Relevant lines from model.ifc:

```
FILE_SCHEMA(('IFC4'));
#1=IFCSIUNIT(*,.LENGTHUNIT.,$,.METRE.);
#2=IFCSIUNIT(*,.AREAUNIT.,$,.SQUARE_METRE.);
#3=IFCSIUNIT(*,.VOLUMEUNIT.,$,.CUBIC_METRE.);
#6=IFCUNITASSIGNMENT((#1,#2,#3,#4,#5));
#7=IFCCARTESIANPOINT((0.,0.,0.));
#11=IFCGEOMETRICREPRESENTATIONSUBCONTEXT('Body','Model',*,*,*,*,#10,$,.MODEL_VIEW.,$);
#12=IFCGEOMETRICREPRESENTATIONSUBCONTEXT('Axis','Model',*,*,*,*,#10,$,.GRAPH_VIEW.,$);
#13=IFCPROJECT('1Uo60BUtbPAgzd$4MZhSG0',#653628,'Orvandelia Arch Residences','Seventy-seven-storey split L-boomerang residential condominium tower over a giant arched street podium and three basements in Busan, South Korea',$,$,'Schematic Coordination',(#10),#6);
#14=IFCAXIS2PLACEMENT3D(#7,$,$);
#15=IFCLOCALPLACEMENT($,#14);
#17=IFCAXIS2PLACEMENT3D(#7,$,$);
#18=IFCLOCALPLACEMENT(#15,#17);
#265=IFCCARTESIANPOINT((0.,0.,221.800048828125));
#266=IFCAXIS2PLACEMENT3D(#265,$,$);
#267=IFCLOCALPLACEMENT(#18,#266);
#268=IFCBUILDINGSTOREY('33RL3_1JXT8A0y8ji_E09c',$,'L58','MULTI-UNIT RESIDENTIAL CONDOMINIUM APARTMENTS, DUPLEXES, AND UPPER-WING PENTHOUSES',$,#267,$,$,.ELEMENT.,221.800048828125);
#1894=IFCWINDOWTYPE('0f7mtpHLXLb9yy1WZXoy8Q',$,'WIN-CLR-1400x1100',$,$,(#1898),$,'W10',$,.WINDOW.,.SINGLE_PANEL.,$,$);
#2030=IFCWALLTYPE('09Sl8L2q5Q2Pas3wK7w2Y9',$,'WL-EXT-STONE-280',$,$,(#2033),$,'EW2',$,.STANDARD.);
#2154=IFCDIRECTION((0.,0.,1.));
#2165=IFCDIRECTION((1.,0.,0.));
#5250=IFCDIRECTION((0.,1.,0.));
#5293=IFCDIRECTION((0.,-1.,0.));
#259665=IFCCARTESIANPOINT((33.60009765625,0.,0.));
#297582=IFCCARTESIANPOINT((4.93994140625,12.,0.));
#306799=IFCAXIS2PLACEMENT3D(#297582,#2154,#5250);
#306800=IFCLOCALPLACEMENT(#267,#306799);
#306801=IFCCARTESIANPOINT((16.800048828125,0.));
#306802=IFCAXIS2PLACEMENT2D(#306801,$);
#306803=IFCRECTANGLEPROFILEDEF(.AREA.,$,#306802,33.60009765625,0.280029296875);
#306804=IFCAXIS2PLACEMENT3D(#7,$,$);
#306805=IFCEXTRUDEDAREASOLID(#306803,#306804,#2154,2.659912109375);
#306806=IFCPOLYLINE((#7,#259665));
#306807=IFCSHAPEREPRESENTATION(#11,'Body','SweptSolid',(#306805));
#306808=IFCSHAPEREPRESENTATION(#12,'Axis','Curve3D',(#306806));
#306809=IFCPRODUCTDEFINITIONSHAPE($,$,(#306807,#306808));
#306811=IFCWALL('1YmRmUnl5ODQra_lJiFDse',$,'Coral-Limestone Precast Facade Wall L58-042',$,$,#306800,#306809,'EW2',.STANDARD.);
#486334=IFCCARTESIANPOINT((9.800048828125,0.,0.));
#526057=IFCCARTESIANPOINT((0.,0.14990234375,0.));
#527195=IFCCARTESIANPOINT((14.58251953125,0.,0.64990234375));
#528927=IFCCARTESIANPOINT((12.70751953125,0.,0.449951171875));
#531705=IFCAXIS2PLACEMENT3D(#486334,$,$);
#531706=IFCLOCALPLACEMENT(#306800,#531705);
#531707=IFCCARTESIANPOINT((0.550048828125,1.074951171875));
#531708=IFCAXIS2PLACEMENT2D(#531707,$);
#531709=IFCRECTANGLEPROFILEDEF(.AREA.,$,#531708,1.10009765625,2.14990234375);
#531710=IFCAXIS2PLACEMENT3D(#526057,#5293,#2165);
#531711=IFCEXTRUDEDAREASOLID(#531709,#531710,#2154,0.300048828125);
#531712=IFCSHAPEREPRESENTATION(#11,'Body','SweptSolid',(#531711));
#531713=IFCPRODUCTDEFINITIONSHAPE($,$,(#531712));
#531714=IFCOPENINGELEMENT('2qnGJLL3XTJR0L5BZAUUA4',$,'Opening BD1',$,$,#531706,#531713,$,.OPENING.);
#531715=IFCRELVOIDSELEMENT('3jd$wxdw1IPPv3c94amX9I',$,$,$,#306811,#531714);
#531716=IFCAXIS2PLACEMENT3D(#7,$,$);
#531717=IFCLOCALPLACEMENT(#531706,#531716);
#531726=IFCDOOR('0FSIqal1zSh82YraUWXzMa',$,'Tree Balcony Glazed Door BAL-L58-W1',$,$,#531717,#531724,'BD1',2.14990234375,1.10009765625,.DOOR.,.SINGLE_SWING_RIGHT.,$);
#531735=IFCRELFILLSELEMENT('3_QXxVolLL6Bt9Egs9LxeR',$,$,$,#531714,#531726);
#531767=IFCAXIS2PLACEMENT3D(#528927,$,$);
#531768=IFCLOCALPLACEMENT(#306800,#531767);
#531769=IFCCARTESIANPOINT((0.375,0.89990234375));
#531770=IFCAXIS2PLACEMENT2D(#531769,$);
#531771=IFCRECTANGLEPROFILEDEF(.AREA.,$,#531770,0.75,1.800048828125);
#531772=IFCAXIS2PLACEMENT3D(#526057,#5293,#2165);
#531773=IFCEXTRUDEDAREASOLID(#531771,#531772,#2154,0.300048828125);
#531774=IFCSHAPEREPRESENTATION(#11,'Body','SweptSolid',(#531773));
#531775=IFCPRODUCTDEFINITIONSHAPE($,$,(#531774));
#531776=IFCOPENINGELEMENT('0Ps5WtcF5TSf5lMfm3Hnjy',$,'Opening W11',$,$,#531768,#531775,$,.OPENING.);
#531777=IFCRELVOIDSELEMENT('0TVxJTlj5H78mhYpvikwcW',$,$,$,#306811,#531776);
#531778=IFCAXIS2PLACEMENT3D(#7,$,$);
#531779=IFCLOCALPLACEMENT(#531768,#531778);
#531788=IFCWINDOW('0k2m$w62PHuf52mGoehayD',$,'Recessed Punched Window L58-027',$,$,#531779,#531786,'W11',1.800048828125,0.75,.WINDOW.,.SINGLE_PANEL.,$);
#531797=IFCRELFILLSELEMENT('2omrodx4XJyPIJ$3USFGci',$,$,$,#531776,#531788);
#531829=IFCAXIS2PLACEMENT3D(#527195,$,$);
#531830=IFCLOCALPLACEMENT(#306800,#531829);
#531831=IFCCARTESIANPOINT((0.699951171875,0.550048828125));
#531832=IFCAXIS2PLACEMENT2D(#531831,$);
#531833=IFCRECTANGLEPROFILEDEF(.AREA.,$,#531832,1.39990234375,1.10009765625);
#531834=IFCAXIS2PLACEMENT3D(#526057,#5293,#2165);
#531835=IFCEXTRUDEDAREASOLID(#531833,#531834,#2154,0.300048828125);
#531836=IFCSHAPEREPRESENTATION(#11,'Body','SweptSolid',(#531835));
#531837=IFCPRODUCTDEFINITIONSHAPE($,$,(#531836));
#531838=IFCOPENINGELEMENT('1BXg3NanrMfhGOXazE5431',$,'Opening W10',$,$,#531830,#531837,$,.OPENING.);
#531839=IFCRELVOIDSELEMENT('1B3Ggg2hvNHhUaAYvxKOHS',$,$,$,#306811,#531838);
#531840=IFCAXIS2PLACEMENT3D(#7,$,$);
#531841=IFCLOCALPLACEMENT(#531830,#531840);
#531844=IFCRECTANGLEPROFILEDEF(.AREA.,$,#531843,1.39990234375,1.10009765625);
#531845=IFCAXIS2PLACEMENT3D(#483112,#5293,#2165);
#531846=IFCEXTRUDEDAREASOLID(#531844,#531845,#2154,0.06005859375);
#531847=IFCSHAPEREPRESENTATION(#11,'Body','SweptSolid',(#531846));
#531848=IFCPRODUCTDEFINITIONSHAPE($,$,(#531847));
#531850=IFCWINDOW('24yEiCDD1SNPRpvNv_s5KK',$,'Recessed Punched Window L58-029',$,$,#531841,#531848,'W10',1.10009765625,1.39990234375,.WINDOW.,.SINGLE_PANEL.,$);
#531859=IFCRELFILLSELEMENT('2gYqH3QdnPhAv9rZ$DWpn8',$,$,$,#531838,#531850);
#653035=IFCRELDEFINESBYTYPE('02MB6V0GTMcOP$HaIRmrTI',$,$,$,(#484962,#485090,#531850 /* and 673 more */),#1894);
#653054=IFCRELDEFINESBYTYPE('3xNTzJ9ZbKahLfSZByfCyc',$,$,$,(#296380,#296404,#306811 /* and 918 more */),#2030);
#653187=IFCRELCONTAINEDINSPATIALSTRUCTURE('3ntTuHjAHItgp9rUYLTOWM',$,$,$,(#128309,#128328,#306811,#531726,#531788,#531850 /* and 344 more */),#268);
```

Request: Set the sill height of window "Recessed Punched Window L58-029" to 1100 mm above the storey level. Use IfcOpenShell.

```python
import numpy as np
import ifcopenshell
import ifcopenshell.api.geometry
import ifcopenshell.geom
import ifcopenshell.util.element
import ifcopenshell.util.placement
import ifcopenshell.util.shape
import ifcopenshell.util.unit

model = ifcopenshell.open("model.ifc")
unit_scale = ifcopenshell.util.unit.calculate_unit_scale(model)

window = model.by_guid("24yEiCDD1SNPRpvNv_s5KK")
opening = window.FillsVoids[0].RelatingOpeningElement
storey = ifcopenshell.util.element.get_container(window, ifc_class="IfcBuildingStorey")
level = ifcopenshell.util.placement.get_local_placement(storey.ObjectPlacement)[2, 3]

# The opening's origin need not be at the sill, so measure its lowest point.
shape = ifcopenshell.geom.create_shape(ifcopenshell.geom.settings(), opening)
bottom = ifcopenshell.util.shape.get_shape_bottom_elevation(shape, shape.geometry) / unit_scale
dz = level + 1.1 / unit_scale - bottom

shift = np.array([0.0, 0.0, dz])
# The window is placed relative to its opening, so it follows when the opening moves.
matrix = ifcopenshell.util.placement.get_local_placement(opening.ObjectPlacement)
matrix[:3, 3] += shift
ifcopenshell.api.geometry.edit_object_placement(
    model, product=opening, matrix=matrix, is_si=False, should_transform_children=True
)

print(f"moved by {dz * unit_scale:+.3f} m")

model.write("model_updated.ifc")
```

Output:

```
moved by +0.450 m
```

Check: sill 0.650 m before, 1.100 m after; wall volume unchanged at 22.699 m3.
